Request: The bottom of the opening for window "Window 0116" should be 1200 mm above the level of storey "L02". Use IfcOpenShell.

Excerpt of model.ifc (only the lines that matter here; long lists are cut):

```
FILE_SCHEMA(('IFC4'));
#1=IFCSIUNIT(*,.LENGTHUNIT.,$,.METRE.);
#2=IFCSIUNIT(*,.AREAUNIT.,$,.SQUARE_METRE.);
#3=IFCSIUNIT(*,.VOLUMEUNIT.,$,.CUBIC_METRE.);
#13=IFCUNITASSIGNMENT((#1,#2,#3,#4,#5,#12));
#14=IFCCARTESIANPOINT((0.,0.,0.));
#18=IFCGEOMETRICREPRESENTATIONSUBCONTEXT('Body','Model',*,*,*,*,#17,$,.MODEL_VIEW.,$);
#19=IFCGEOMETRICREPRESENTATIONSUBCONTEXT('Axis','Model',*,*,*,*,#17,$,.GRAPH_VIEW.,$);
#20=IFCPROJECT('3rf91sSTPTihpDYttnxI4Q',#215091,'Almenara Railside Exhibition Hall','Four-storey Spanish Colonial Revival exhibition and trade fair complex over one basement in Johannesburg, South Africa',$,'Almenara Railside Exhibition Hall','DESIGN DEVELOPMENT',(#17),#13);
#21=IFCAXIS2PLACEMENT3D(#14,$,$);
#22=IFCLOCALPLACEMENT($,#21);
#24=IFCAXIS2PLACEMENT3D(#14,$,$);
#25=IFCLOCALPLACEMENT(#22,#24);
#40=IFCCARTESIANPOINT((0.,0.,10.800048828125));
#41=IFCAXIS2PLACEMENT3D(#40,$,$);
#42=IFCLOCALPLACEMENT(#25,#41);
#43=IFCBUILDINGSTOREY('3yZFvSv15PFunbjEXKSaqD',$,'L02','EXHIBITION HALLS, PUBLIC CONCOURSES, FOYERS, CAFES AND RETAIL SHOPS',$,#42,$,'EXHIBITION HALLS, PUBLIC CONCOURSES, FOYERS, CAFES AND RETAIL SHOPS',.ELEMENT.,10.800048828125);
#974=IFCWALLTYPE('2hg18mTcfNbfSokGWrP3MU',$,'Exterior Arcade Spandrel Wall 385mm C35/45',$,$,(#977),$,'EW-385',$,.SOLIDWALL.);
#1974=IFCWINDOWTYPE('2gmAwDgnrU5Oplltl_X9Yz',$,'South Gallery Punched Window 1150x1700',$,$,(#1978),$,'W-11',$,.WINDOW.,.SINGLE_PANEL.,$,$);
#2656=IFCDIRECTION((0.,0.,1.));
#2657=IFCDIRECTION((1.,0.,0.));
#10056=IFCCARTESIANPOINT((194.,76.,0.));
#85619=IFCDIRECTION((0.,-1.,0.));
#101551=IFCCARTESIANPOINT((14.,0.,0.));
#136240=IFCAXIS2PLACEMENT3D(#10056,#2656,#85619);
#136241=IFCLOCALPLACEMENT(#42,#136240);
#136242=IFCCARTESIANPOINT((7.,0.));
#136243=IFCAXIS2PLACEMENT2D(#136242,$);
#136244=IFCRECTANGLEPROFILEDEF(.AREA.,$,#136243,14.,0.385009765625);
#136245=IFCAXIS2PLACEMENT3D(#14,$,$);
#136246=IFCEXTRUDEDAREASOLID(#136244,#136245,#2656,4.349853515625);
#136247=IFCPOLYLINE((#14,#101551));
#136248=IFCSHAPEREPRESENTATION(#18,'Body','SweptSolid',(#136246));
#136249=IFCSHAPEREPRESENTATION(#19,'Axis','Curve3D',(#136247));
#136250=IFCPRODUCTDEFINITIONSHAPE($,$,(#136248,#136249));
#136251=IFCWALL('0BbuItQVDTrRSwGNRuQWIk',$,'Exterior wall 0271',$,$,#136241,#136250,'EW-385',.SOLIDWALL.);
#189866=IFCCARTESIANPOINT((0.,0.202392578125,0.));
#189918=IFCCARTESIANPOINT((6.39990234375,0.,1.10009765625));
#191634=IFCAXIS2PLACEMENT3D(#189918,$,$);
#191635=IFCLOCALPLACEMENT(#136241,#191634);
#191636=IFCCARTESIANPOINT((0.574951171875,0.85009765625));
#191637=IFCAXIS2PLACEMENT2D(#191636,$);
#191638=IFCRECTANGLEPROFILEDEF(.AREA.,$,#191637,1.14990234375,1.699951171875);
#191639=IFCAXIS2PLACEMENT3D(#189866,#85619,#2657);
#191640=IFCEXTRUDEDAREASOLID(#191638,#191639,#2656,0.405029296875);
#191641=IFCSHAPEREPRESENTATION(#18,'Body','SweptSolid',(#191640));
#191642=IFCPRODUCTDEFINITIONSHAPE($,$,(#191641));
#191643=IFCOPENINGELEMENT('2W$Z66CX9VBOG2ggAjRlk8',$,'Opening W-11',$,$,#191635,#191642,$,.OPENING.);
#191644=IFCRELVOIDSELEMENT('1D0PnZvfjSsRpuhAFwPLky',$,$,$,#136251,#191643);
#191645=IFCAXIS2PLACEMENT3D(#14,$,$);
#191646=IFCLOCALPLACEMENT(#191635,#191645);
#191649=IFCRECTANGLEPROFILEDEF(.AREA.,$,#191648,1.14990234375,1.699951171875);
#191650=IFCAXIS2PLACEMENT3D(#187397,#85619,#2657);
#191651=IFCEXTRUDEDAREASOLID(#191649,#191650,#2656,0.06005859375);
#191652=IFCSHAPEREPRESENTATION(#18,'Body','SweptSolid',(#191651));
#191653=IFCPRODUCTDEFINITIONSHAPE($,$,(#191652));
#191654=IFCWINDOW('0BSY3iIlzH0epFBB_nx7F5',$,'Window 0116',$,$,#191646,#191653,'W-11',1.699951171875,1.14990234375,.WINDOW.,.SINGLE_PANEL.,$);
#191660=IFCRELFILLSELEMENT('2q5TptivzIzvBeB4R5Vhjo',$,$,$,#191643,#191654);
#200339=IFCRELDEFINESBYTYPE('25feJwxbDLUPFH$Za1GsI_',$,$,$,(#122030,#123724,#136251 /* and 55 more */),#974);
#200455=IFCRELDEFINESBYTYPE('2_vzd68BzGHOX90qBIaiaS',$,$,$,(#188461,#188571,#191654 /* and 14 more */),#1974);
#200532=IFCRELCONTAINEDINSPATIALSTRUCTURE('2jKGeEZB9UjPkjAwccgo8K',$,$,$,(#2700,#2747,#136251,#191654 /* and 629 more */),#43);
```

```python
import numpy as np
import ifcopenshell
import ifcopenshell.api.geometry
import ifcopenshell.geom
import ifcopenshell.util.element
import ifcopenshell.util.placement
import ifcopenshell.util.shape
import ifcopenshell.util.unit

model = ifcopenshell.open("model.ifc")
unit_scale = ifcopenshell.util.unit.calculate_unit_scale(model)

window = model.by_guid("0BSY3iIlzH0epFBB_nx7F5")
opening = window.FillsVoids[0].RelatingOpeningElement
storey = ifcopenshell.util.element.get_container(window, ifc_class="IfcBuildingStorey")
level = ifcopenshell.util.placement.get_local_placement(storey.ObjectPlacement)[2, 3]

# The opening's origin need not be at the sill, so measure its lowest point.
shape = ifcopenshell.geom.create_shape(ifcopenshell.geom.settings(), opening)
bottom = ifcopenshell.util.shape.get_shape_bottom_elevation(shape, shape.geometry) / unit_scale
dz = level + 1.2 - bottom

shift = np.array([0.0, 0.0, dz])
# The window is placed relative to its opening, so it follows when the opening moves.
matrix = ifcopenshell.util.placement.get_local_placement(opening.ObjectPlacement)
matrix[:3, 3] += shift
ifcopenshell.api.geometry.edit_object_placement(
    model, product=opening, matrix=matrix, is_si=False, should_transform_children=True
)

print(f"moved by {dz * unit_scale:+.3f} m")

model.write("model_v2.ifc")
```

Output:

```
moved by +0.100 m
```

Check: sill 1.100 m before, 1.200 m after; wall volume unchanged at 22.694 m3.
